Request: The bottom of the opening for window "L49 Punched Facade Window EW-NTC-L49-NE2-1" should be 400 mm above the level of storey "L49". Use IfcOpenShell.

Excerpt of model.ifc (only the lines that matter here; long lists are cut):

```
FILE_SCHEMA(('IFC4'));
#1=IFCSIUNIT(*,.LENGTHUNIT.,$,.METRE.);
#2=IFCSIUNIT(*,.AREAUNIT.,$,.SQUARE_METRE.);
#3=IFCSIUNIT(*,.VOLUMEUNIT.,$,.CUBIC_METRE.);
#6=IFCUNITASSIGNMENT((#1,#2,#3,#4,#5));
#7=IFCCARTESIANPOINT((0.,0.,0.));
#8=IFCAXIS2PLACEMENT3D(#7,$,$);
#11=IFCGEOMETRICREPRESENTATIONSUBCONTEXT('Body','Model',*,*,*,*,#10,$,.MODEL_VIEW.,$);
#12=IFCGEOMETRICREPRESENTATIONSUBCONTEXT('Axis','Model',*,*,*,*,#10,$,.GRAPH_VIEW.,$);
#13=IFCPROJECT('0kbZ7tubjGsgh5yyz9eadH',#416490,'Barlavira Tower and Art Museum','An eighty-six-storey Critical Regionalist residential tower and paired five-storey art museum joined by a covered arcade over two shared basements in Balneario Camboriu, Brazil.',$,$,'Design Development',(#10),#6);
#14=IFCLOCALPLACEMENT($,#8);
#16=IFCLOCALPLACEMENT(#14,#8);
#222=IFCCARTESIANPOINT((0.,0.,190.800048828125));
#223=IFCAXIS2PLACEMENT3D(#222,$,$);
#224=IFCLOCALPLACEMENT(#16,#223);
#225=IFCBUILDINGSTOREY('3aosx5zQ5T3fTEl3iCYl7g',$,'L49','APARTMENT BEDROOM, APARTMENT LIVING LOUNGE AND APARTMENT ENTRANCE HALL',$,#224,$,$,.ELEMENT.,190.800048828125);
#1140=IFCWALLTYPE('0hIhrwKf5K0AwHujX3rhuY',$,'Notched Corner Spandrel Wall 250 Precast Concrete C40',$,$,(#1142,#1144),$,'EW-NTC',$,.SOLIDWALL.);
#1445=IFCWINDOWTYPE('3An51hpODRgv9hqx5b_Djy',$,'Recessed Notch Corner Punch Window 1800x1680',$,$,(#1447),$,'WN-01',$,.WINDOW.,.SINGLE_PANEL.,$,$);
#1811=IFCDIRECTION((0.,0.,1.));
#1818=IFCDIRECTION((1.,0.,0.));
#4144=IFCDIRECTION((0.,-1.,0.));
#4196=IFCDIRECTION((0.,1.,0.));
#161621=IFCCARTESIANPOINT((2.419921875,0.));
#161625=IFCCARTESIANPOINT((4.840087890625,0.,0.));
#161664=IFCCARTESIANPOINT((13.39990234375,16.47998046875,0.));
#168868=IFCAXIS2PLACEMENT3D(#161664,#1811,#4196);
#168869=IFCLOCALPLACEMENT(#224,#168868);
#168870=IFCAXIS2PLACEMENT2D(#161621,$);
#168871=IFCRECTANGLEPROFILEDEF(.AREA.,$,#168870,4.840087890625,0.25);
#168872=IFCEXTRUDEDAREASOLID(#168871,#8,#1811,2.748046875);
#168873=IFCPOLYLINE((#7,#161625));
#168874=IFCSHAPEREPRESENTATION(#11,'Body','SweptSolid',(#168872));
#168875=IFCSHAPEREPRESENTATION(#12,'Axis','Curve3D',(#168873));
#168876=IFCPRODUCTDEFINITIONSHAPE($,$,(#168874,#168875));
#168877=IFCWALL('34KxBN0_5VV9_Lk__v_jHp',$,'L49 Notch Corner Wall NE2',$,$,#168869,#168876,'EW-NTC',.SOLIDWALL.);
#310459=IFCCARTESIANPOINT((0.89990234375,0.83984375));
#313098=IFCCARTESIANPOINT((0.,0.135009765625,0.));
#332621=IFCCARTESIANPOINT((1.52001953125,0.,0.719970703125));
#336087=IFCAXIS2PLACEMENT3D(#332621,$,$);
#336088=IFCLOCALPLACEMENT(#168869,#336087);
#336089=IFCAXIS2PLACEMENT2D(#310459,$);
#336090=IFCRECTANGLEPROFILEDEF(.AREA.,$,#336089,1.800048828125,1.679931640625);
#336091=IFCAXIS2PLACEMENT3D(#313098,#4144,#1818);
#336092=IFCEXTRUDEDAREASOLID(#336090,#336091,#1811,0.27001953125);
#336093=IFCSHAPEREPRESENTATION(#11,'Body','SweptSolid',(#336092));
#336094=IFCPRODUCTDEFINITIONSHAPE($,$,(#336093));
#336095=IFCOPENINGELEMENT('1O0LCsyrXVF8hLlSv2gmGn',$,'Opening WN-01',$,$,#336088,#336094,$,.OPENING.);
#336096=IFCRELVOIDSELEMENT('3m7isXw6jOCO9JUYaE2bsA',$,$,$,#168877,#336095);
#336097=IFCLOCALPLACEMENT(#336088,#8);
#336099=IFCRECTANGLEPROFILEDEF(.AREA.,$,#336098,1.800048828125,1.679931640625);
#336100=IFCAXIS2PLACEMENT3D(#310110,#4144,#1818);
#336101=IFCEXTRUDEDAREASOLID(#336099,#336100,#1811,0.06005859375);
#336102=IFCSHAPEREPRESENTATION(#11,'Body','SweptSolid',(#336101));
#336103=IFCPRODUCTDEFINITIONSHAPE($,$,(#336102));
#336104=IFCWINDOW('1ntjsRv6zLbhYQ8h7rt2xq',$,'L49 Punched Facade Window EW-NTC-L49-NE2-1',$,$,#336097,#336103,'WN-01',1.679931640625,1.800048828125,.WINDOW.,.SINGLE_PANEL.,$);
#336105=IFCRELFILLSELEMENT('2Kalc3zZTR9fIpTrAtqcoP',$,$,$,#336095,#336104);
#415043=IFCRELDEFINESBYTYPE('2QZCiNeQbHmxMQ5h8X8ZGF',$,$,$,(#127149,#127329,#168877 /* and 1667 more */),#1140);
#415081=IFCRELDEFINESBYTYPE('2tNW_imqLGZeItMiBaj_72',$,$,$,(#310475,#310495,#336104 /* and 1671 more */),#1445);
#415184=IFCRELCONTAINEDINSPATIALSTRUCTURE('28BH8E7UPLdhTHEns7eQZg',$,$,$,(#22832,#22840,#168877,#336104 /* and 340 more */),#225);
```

```python
import numpy as np
import ifcopenshell
import ifcopenshell.api.geometry
import ifcopenshell.geom
import ifcopenshell.util.element
import ifcopenshell.util.placement
import ifcopenshell.util.shape
import ifcopenshell.util.unit

model = ifcopenshell.open("model.ifc")
unit_scale = ifcopenshell.util.unit.calculate_unit_scale(model)

window = model.by_guid("1ntjsRv6zLbhYQ8h7rt2xq")
opening = window.FillsVoids[0].RelatingOpeningElement
storey = ifcopenshell.util.element.get_container(window, ifc_class="IfcBuildingStorey")
level = ifcopenshell.util.placement.get_local_placement(storey.ObjectPlacement)[2, 3]

# The opening's origin need not be at the sill, so measure its lowest point.
shape = ifcopenshell.geom.create_shape(ifcopenshell.geom.settings(), opening)
bottom = ifcopenshell.util.shape.get_shape_bottom_elevation(shape, shape.geometry) / unit_scale
dz = level + 0.4 / unit_scale - bottom

shift = np.array([0.0, 0.0, dz])
# The window is placed relative to its opening, so it follows when the opening moves.
matrix = ifcopenshell.util.placement.get_local_placement(opening.ObjectPlacement)
matrix[:3, 3] += shift
ifcopenshell.api.geometry.edit_object_placement(
    model, product=opening, matrix=matrix, is_si=False, should_transform_children=True
)

print(f"moved by {dz * unit_scale:+.3f} m")

model.write("model-out.ifc")
```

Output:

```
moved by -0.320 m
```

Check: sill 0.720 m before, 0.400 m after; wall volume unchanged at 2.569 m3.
